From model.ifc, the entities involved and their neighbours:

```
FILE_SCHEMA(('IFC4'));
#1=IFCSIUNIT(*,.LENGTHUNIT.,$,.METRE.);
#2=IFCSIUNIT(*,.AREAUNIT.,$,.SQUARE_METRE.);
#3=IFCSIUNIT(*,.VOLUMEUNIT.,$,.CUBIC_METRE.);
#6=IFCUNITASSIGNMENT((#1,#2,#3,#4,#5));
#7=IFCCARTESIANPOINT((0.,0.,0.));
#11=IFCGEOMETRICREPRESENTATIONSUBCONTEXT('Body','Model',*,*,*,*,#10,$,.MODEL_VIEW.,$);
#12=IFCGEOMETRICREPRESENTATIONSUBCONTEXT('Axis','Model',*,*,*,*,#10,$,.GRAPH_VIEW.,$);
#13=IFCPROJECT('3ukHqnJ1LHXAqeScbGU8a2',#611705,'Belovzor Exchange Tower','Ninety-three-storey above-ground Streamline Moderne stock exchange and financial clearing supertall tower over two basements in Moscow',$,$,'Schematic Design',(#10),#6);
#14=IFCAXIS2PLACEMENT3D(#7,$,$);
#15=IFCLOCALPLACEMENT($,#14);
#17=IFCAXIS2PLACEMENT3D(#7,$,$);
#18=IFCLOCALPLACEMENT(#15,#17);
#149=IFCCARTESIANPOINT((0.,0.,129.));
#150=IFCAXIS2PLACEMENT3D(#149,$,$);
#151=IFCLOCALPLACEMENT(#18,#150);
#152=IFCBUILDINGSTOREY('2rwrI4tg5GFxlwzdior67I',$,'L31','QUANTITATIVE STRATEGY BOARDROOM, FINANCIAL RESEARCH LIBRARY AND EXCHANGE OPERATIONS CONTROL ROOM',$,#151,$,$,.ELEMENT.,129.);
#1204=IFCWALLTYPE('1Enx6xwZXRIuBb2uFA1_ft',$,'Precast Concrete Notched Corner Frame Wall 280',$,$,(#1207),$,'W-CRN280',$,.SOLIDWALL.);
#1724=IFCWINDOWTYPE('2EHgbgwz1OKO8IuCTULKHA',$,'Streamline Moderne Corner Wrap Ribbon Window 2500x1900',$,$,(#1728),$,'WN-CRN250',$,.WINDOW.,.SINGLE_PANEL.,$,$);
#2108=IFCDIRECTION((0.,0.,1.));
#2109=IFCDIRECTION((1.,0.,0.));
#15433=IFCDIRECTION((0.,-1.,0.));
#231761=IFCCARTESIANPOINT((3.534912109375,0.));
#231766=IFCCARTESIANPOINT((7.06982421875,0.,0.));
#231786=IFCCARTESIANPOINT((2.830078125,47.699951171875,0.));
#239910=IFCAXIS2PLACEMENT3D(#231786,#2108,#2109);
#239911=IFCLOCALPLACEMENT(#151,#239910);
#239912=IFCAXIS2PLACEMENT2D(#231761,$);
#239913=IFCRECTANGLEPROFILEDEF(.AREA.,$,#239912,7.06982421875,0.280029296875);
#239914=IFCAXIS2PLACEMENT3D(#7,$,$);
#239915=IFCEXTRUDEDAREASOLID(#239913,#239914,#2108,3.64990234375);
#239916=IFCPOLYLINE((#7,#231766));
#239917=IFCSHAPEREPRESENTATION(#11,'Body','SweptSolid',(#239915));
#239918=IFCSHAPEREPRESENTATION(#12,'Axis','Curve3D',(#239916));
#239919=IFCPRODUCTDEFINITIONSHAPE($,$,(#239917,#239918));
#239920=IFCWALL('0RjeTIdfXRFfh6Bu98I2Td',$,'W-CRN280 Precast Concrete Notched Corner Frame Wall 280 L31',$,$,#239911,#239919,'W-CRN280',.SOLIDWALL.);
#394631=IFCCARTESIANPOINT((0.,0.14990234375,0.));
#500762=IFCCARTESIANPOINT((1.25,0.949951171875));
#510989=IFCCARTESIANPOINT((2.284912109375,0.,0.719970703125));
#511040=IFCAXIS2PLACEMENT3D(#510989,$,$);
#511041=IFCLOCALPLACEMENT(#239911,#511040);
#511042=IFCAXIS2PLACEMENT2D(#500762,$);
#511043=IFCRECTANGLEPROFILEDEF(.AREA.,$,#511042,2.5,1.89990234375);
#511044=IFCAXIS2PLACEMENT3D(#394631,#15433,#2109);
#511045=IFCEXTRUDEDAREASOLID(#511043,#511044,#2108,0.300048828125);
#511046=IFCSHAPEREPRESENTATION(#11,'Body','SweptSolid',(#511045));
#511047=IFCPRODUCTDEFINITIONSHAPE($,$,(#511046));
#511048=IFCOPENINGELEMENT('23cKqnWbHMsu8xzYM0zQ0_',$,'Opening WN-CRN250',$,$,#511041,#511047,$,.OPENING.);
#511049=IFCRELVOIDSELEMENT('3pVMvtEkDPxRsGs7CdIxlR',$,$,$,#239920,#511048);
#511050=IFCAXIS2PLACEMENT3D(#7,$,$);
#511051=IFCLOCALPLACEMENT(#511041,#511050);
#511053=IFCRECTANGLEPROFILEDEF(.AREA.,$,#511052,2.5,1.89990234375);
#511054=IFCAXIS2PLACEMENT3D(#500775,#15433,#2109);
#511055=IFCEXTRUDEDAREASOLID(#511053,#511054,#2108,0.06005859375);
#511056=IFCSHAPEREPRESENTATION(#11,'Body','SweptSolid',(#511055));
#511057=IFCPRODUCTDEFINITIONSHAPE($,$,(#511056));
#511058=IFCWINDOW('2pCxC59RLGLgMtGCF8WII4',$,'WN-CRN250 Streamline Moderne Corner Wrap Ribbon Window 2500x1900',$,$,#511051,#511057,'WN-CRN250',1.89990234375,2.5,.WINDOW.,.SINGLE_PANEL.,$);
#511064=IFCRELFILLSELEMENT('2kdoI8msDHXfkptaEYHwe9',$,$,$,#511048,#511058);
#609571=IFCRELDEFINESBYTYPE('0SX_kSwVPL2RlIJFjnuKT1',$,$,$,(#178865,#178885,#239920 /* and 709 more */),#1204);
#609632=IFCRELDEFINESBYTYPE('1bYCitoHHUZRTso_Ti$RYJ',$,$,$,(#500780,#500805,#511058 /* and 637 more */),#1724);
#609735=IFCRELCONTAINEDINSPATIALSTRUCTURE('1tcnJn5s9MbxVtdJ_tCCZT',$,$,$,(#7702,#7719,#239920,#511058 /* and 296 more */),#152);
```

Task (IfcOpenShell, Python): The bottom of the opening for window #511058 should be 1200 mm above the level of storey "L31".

```python
import numpy as np
import ifcopenshell
import ifcopenshell.api.geometry
import ifcopenshell.geom
import ifcopenshell.util.element
import ifcopenshell.util.placement
import ifcopenshell.util.shape
import ifcopenshell.util.unit

model = ifcopenshell.open("model.ifc")
unit_scale = ifcopenshell.util.unit.calculate_unit_scale(model)

window = model.by_guid("2pCxC59RLGLgMtGCF8WII4")
opening = window.FillsVoids[0].RelatingOpeningElement
storey = ifcopenshell.util.element.get_container(window, ifc_class="IfcBuildingStorey")
level = ifcopenshell.util.placement.get_local_placement(storey.ObjectPlacement)[2, 3]

# The opening's origin need not be at the sill, so measure its lowest point.
shape = ifcopenshell.geom.create_shape(ifcopenshell.geom.settings(), opening)
bottom = ifcopenshell.util.shape.get_shape_bottom_elevation(shape, shape.geometry) / unit_scale
dz = level + 1.2 / unit_scale - bottom

shift = np.array([0.0, 0.0, dz])
# The window is placed relative to its opening, so it follows when the opening moves.
matrix = ifcopenshell.util.placement.get_local_placement(opening.ObjectPlacement)
matrix[:3, 3] += shift
ifcopenshell.api.geometry.edit_object_placement(
    model, product=opening, matrix=matrix, is_si=False, should_transform_children=True
)

print(f"moved by {dz * unit_scale:+.3f} m")

model.write("model_v2.ifc")
```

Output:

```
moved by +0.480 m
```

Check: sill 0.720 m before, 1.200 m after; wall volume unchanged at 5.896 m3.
